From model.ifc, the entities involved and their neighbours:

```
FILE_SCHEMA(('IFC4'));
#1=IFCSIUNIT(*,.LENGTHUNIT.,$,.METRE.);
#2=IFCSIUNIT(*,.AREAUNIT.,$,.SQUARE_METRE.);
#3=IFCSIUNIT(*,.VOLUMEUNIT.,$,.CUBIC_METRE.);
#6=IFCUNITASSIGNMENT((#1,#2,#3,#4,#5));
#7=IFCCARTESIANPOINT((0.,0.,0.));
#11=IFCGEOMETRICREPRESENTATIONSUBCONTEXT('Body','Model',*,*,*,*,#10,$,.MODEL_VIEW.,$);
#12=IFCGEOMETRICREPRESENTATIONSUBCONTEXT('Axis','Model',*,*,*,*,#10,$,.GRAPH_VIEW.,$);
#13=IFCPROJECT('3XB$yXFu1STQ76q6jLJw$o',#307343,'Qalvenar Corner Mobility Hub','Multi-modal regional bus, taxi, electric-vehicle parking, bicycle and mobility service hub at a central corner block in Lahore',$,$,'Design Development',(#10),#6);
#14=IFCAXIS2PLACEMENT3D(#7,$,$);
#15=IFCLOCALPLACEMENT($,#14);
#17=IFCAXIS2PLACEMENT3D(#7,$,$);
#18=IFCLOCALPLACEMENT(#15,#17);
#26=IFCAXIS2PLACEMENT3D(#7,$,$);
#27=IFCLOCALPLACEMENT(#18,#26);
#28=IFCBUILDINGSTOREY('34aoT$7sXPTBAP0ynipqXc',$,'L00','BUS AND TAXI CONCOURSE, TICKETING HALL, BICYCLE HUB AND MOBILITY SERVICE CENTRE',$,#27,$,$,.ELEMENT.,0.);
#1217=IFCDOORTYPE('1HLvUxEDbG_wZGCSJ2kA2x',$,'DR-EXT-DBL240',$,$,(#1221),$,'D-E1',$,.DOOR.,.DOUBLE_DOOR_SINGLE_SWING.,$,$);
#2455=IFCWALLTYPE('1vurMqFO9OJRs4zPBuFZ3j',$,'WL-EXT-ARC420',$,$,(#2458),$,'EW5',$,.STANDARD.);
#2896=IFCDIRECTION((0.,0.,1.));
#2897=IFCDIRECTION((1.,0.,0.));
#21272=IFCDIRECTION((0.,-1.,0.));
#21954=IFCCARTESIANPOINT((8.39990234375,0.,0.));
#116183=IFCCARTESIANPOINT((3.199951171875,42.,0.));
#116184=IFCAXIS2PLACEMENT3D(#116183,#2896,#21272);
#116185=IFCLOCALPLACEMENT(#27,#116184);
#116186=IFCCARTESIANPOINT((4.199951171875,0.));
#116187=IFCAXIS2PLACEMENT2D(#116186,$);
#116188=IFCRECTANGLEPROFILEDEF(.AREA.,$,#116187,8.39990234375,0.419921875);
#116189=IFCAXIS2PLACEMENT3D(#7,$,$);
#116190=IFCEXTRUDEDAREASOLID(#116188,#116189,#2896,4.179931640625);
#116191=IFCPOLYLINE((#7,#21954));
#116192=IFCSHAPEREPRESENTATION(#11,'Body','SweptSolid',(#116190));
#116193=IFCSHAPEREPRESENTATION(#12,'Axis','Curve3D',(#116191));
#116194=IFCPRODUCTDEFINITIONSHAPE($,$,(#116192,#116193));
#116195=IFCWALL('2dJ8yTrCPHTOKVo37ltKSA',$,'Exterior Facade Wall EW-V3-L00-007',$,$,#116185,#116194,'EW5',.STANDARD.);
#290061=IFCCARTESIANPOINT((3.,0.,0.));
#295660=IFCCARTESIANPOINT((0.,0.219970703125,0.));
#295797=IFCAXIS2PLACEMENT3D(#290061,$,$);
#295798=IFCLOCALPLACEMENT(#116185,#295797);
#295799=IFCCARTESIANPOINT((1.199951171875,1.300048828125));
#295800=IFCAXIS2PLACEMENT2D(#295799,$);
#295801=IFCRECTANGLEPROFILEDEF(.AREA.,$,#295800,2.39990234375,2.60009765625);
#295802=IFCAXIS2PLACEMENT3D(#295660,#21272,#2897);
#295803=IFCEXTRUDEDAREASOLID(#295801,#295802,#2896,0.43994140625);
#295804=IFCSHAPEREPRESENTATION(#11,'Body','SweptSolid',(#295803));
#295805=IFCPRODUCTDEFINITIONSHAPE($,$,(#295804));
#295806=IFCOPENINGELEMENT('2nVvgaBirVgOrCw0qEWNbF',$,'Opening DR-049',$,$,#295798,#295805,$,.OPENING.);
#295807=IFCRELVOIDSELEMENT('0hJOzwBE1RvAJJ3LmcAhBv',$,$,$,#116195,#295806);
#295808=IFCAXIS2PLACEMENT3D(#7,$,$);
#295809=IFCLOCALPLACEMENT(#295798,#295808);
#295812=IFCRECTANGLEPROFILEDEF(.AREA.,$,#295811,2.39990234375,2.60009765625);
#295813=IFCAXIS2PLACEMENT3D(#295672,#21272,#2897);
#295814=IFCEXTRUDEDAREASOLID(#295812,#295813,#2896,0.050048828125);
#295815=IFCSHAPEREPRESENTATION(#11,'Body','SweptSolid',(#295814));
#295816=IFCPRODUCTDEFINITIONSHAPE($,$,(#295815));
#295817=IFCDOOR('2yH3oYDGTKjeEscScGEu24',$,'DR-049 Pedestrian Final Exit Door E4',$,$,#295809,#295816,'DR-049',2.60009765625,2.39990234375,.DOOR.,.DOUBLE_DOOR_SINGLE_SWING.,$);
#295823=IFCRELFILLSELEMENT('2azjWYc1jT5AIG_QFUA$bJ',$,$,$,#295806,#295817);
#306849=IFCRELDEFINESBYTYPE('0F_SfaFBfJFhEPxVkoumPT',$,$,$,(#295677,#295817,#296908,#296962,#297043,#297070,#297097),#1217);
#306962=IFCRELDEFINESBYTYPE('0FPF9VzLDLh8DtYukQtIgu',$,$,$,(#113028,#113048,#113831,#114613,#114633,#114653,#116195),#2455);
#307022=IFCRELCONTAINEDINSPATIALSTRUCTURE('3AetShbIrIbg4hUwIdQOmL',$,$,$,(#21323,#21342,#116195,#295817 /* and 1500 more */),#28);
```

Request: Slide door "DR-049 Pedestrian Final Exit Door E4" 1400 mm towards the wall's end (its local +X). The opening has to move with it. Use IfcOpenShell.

```python
import ifcopenshell
import ifcopenshell.api.geometry
import ifcopenshell.util.placement
import ifcopenshell.util.unit

model = ifcopenshell.open("model.ifc")
unit_scale = ifcopenshell.util.unit.calculate_unit_scale(model)

door = model.by_guid("2yH3oYDGTKjeEscScGEu24")
opening = door.FillsVoids[0].RelatingOpeningElement
wall = opening.VoidsElements[0].RelatingBuildingElement

wall_matrix = ifcopenshell.util.placement.get_local_placement(wall.ObjectPlacement)
shift = wall_matrix[:3, 0] * 1.4 / unit_scale
before = ifcopenshell.util.placement.get_local_placement(door.ObjectPlacement)[:3, 3].copy()

# The door is placed relative to its opening, so it follows when the opening moves.
matrix = ifcopenshell.util.placement.get_local_placement(opening.ObjectPlacement)
matrix[:3, 3] += shift
ifcopenshell.api.geometry.edit_object_placement(
    model, product=opening, matrix=matrix, is_si=False, should_transform_children=True
)

after = ifcopenshell.util.placement.get_local_placement(door.ObjectPlacement)[:3, 3]
print("door moved by", (after - before).round(3) + 0.0)

model.write("model_rev.ifc")
```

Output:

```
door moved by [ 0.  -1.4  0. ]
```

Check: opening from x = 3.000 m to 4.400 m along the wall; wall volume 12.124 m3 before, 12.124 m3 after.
